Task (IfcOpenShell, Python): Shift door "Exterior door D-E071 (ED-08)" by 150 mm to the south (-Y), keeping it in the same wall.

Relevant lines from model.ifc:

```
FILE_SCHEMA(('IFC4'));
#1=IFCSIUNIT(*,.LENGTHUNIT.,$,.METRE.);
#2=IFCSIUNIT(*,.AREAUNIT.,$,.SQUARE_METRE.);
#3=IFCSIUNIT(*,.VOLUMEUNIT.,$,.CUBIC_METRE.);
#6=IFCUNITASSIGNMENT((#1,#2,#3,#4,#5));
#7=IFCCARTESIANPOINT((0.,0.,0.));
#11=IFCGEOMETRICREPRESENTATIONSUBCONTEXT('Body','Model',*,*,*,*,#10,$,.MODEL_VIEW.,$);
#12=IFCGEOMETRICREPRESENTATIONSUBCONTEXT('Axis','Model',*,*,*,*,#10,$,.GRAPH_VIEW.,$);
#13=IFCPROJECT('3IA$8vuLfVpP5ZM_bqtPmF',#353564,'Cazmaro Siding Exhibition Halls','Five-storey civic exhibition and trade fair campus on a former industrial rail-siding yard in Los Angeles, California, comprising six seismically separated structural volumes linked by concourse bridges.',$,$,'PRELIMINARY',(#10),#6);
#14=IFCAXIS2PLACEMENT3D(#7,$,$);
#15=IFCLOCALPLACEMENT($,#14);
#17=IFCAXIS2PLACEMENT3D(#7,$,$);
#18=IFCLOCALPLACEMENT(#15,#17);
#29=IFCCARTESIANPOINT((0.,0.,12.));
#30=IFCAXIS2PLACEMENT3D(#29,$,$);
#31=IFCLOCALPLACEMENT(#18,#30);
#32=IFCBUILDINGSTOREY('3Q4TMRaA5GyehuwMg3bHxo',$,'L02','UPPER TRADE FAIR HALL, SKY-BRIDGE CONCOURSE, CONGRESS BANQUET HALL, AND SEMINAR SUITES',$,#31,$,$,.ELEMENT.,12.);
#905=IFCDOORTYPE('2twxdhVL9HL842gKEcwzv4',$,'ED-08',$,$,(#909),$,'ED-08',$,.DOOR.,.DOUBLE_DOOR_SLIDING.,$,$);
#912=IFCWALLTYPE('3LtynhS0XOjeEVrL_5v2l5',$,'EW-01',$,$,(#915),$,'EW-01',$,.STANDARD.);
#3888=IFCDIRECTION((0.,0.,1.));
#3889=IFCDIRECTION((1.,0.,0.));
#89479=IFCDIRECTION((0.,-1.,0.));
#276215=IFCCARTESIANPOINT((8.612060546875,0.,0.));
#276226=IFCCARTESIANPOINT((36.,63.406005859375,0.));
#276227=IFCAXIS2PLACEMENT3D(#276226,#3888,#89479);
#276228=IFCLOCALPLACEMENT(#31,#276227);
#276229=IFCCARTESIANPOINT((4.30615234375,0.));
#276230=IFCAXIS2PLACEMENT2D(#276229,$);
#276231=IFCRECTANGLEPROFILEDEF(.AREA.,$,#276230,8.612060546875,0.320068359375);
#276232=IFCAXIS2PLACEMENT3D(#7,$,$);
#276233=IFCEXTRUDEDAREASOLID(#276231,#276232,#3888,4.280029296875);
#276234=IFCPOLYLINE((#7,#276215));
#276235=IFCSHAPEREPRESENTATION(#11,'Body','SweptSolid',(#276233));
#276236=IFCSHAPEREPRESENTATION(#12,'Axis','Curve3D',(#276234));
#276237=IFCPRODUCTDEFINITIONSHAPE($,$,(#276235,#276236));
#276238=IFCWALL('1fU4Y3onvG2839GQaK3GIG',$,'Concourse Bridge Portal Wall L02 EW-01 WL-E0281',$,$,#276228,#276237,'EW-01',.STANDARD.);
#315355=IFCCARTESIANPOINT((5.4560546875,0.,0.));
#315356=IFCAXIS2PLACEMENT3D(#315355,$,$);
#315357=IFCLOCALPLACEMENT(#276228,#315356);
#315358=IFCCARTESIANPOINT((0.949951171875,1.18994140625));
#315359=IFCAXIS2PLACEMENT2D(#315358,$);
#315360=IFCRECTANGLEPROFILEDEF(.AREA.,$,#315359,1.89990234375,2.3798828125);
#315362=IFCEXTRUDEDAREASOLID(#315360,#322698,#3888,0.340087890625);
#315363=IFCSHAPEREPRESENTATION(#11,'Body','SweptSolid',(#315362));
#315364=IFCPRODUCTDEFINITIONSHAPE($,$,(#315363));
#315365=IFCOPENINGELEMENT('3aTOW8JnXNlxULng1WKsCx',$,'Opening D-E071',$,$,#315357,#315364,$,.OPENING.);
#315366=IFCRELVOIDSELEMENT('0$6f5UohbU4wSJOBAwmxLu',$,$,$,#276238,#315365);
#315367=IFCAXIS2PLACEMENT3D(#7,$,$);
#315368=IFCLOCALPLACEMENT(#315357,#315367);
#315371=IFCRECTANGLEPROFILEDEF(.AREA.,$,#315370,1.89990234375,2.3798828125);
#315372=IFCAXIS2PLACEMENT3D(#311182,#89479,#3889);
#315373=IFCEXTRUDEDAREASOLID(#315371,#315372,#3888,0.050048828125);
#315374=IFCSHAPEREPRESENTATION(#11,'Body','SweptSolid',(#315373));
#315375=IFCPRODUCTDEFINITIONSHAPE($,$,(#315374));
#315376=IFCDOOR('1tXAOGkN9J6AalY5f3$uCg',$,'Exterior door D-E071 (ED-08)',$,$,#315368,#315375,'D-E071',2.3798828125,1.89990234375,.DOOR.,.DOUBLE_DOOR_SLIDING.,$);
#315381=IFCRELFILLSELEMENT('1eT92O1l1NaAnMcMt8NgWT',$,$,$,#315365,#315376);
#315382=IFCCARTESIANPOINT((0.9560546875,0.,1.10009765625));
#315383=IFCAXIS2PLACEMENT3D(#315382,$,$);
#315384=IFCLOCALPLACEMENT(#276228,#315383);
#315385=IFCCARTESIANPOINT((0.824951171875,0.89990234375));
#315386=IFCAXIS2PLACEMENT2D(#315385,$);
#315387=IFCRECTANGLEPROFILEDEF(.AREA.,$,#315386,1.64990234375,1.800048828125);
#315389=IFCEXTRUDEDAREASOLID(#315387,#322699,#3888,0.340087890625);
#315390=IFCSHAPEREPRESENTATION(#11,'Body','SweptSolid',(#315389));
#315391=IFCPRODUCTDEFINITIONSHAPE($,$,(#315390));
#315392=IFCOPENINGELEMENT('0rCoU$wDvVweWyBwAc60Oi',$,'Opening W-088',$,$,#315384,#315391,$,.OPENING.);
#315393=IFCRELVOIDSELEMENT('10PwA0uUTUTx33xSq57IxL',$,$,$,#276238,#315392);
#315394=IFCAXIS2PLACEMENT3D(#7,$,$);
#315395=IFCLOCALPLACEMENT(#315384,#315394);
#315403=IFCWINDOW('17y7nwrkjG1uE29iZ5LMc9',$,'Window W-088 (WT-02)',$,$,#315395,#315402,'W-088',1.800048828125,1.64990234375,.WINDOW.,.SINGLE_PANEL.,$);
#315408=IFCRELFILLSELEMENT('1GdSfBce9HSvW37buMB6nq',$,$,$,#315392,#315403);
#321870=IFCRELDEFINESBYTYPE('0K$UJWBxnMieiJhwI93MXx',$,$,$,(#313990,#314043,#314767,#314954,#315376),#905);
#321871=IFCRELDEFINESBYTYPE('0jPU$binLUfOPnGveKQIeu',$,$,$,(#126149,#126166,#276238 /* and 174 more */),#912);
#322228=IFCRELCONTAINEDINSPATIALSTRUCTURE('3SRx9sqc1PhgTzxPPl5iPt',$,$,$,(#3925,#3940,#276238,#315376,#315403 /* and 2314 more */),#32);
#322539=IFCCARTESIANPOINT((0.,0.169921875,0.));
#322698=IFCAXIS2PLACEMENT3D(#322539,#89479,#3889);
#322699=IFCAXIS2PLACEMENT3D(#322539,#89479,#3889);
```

```python
import ifcopenshell
import ifcopenshell.api.geometry
import ifcopenshell.util.placement
import ifcopenshell.util.unit

model = ifcopenshell.open("model.ifc")
unit_scale = ifcopenshell.util.unit.calculate_unit_scale(model)

door = model.by_guid("1tXAOGkN9J6AalY5f3$uCg")
opening = door.FillsVoids[0].RelatingOpeningElement
wall = opening.VoidsElements[0].RelatingBuildingElement

wall_matrix = ifcopenshell.util.placement.get_local_placement(wall.ObjectPlacement)
shift = wall_matrix[:3, 0] * 0.15 / unit_scale
before = ifcopenshell.util.placement.get_local_placement(door.ObjectPlacement)[:3, 3].copy()

# The door is placed relative to its opening, so it follows when the opening moves.
matrix = ifcopenshell.util.placement.get_local_placement(opening.ObjectPlacement)
matrix[:3, 3] += shift
ifcopenshell.api.geometry.edit_object_placement(
    model, product=opening, matrix=matrix, is_si=False, should_transform_children=True
)

after = ifcopenshell.util.placement.get_local_placement(door.ObjectPlacement)[:3, 3]
print("door moved by", (after - before).round(3) + 0.0)

model.write("model_rev.ifc")
```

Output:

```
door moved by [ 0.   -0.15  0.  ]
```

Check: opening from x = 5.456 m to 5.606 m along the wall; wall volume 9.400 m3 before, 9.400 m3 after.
